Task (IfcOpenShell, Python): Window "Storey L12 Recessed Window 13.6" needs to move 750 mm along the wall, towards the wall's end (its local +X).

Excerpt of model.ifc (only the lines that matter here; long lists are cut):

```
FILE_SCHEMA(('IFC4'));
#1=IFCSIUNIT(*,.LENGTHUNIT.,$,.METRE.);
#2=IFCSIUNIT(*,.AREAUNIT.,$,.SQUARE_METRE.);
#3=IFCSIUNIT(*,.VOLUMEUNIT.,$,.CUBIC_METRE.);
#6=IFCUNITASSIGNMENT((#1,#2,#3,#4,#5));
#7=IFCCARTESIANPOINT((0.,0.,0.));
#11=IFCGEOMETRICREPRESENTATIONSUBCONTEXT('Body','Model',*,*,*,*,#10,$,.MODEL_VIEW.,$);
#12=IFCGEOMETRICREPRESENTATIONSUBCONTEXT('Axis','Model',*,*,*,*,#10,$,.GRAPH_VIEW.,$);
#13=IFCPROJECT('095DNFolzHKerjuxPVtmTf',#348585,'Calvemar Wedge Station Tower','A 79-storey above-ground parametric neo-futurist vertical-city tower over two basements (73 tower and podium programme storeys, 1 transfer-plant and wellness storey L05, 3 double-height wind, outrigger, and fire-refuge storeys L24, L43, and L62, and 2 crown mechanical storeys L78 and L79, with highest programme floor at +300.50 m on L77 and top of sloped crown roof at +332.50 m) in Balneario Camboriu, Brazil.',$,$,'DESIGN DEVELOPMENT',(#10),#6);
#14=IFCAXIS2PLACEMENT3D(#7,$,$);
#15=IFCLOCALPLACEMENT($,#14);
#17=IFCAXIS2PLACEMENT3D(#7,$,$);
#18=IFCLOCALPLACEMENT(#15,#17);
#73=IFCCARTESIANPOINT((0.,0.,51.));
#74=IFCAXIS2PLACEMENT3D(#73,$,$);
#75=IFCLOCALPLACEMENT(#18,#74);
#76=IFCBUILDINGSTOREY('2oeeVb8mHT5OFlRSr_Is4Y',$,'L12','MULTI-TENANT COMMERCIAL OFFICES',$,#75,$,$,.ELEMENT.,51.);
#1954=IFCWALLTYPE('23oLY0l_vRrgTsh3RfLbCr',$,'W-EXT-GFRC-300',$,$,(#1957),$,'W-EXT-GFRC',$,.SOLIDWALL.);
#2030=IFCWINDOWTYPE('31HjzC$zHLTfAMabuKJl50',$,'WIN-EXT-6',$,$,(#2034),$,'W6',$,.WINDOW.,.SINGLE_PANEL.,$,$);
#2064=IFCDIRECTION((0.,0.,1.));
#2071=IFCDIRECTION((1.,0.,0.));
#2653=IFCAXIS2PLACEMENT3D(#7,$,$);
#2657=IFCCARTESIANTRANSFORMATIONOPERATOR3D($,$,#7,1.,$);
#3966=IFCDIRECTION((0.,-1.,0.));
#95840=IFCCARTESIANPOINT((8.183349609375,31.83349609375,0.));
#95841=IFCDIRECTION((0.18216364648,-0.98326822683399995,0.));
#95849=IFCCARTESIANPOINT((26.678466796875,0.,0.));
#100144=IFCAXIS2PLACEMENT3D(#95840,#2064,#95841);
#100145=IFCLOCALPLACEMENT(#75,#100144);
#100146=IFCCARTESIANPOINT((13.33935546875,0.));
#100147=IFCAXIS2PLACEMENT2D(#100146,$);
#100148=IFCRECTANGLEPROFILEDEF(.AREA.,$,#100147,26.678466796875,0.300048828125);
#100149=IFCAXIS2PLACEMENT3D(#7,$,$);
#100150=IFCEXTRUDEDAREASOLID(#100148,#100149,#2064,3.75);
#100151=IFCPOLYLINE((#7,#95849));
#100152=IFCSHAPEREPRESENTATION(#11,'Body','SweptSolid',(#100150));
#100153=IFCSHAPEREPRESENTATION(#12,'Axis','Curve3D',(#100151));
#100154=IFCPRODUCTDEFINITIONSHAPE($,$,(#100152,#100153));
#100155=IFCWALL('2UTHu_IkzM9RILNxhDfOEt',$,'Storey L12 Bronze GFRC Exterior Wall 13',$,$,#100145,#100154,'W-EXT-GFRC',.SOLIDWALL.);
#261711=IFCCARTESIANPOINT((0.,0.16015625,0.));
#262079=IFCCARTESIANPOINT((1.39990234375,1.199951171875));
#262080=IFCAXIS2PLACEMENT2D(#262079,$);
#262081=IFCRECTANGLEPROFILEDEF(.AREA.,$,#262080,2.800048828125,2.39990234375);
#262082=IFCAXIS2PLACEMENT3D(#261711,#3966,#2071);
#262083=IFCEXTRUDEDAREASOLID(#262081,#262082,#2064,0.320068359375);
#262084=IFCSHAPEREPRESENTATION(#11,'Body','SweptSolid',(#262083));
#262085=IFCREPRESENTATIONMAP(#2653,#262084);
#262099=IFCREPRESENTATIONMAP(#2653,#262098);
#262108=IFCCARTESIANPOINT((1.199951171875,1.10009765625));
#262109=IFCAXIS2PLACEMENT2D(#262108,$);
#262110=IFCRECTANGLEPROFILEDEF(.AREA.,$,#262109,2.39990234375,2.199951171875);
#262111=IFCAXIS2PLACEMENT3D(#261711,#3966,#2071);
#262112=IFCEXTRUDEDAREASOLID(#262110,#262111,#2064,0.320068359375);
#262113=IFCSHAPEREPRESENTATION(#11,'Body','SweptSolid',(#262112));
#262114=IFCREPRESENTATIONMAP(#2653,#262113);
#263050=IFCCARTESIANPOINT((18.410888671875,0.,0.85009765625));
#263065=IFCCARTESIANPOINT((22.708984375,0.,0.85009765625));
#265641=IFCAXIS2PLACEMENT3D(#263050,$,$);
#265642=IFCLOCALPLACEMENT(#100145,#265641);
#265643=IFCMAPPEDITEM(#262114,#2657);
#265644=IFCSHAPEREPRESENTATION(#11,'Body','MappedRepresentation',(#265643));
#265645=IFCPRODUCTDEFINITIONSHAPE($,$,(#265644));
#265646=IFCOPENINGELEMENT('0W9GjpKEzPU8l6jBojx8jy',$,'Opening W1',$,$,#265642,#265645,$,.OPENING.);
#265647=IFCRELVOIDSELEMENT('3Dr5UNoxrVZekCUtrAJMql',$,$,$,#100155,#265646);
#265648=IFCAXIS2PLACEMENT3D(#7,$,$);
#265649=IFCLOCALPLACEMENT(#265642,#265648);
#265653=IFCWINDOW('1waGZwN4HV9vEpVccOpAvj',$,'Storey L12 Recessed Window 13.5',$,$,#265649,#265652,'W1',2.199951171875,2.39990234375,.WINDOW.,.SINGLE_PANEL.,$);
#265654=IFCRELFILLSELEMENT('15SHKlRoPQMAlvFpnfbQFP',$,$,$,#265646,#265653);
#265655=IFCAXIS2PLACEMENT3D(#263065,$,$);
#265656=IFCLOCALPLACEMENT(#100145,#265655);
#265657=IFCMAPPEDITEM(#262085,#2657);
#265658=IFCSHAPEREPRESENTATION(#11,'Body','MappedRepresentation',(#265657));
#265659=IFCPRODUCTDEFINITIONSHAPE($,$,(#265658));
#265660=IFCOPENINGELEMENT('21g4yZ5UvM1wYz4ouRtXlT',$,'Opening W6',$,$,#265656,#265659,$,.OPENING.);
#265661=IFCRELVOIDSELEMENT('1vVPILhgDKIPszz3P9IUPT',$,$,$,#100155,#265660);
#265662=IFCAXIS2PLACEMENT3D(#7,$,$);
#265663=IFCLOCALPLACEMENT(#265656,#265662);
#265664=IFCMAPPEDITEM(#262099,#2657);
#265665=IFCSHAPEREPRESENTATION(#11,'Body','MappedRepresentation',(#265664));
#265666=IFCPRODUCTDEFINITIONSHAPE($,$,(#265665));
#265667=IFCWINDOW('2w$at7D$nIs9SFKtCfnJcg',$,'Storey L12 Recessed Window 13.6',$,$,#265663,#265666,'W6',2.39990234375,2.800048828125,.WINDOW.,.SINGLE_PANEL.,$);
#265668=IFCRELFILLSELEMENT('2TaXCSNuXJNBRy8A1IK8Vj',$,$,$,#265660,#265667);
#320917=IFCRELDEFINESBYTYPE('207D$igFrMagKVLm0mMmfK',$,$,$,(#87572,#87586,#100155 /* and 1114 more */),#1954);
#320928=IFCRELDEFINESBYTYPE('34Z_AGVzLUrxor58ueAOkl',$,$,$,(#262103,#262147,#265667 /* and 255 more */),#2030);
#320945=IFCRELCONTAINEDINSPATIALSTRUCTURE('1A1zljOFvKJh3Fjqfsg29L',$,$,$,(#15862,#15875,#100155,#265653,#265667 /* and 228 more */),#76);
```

```python
import ifcopenshell
import ifcopenshell.api.geometry
import ifcopenshell.util.placement

model = ifcopenshell.open("model.ifc")

window = model.by_guid("2w$at7D$nIs9SFKtCfnJcg")
opening = window.FillsVoids[0].RelatingOpeningElement
wall = opening.VoidsElements[0].RelatingBuildingElement

wall_matrix = ifcopenshell.util.placement.get_local_placement(wall.ObjectPlacement)
shift = wall_matrix[:3, 0] * 0.75
before = ifcopenshell.util.placement.get_local_placement(window.ObjectPlacement)[:3, 3].copy()

# The window is placed relative to its opening, so it follows when the opening moves.
matrix = ifcopenshell.util.placement.get_local_placement(opening.ObjectPlacement)
matrix[:3, 3] += shift
ifcopenshell.api.geometry.edit_object_placement(
    model, product=opening, matrix=matrix, is_si=False, should_transform_children=True
)

after = ifcopenshell.util.placement.get_local_placement(window.ObjectPlacement)[:3, 3]
print("window moved by", (after - before).round(3) + 0.0)

model.write("model_v2.ifc")
```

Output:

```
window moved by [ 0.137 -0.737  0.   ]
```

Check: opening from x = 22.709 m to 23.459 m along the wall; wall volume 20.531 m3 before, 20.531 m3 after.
